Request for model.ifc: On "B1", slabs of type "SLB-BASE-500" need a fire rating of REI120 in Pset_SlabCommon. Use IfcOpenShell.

First a look at what the model holds.

```python
import ifcopenshell
import ifcopenshell.util.element

model = ifcopenshell.open("model.ifc")
print(model.schema)
storey = next(s for s in model.by_type("IfcBuildingStorey") if s.Name == "B1")
slabs = [e for e in ifcopenshell.util.element.get_decomposition(storey) if e.is_a("IfcSlab")]
seen = {}
for e in slabs:
    element_type = ifcopenshell.util.element.get_type(e)
    key = (element_type.Name if element_type != e and element_type else None, ifcopenshell.util.element.get_pset(e, "Pset_SlabCommon", "FireRating"))
    seen[key] = seen.get(key, 0) + 1
for (name, value), count in sorted(seen.items(), key=str):
    print(count, "x", name, "|", value)
```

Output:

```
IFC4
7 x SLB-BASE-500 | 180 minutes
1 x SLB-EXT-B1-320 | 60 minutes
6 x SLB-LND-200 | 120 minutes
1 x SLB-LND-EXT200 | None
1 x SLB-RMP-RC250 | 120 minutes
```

```python
import ifcopenshell
import ifcopenshell.api.pset
import ifcopenshell.util.element

model = ifcopenshell.open("model.ifc")

storey = next(s for s in model.by_type("IfcBuildingStorey") if s.Name == "B1")
slabs = [e for e in ifcopenshell.util.element.get_decomposition(storey) if e.is_a("IfcSlab")]

count = 0
for e in slabs:
    element_type = ifcopenshell.util.element.get_type(e)
    if element_type in (None, e) or element_type.Name != "SLB-BASE-500":
        continue
    # add_pset returns the element's existing set when there is one.
    pset = ifcopenshell.api.pset.add_pset(model, product=e, name="Pset_SlabCommon")
    ifcopenshell.api.pset.edit_pset(model, pset=pset, properties={"FireRating": "REI120"})
    count += 1

print(count, "slabs updated")

model.write("model_rev.ifc")
```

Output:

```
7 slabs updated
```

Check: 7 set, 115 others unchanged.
